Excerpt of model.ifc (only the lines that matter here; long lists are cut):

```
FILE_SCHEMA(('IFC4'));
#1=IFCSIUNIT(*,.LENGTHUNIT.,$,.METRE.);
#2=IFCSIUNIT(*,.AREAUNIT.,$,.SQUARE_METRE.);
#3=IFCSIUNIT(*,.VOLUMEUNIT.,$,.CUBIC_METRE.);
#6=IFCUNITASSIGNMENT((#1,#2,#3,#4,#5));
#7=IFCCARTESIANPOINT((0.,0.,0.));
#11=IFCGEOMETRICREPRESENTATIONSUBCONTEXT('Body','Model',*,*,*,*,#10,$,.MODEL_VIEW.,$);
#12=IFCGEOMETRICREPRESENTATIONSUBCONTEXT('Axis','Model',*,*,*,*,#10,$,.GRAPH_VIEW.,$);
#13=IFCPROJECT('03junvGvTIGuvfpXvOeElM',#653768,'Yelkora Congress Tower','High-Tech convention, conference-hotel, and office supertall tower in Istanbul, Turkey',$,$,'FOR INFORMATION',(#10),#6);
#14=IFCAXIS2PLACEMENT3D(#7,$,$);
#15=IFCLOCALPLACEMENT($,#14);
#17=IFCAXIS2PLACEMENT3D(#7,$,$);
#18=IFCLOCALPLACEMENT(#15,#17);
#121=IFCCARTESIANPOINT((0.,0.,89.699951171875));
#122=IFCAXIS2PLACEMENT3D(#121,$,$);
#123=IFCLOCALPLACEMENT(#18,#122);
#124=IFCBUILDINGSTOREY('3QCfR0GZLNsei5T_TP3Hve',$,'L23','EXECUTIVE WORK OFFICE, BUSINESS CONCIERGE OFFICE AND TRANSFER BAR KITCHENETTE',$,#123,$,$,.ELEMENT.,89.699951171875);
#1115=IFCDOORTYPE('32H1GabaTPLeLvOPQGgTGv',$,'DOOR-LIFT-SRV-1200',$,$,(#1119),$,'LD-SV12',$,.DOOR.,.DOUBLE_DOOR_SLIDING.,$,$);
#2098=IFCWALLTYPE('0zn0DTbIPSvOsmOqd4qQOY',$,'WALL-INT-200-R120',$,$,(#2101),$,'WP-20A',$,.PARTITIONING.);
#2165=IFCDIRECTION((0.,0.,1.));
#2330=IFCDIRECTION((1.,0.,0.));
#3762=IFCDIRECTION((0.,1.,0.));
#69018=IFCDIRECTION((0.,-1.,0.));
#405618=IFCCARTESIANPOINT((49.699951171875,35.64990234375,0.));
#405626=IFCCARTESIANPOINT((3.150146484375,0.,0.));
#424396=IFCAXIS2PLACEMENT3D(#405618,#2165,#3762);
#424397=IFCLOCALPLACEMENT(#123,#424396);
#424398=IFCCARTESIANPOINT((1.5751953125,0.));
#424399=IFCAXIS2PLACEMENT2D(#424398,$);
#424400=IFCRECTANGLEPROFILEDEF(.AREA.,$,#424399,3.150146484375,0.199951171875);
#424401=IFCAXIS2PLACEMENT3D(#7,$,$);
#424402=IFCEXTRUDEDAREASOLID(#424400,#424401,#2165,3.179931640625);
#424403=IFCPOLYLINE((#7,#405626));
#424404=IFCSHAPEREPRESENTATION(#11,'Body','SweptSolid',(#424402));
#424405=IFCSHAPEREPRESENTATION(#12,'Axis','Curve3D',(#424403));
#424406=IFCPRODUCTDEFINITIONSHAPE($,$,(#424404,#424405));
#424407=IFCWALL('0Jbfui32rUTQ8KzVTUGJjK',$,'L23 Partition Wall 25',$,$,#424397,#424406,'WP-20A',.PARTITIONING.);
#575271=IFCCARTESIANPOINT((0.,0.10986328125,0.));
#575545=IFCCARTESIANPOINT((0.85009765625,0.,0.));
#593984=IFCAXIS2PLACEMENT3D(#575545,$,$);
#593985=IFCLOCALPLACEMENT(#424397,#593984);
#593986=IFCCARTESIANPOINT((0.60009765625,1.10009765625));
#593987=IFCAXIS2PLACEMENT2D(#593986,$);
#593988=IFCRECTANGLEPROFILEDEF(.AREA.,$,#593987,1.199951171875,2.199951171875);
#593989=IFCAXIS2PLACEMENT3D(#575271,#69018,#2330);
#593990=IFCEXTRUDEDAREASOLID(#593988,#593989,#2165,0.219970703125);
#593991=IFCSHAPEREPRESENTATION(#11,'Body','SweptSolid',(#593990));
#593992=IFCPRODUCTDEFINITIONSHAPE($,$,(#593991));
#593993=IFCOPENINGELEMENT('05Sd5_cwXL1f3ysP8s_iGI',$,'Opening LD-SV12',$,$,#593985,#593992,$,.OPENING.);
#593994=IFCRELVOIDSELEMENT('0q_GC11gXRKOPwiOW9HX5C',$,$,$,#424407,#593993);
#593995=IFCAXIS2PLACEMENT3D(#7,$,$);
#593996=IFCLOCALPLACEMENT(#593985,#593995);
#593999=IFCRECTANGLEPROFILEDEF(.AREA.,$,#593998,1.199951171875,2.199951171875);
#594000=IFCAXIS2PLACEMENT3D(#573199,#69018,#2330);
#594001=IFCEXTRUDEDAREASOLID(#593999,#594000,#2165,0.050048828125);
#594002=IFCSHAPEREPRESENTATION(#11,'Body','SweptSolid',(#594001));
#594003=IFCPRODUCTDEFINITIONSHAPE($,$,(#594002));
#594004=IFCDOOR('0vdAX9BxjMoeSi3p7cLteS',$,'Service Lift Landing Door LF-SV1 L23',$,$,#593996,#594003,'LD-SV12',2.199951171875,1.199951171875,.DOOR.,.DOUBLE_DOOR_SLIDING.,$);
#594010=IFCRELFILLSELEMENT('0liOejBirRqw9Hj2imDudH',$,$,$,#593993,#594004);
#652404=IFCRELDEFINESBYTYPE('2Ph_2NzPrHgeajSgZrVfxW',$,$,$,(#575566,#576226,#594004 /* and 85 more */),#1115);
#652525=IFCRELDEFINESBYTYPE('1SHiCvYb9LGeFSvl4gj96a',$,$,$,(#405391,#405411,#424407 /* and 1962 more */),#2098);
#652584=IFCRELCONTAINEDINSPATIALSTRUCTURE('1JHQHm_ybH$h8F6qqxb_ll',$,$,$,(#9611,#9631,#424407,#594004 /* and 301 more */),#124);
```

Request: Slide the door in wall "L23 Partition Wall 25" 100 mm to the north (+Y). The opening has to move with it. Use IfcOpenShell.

```python
import ifcopenshell
import ifcopenshell.api.geometry
import ifcopenshell.util.placement

model = ifcopenshell.open("model.ifc")

door = model.by_guid("0vdAX9BxjMoeSi3p7cLteS")
opening = door.FillsVoids[0].RelatingOpeningElement
wall = opening.VoidsElements[0].RelatingBuildingElement

wall_matrix = ifcopenshell.util.placement.get_local_placement(wall.ObjectPlacement)
shift = wall_matrix[:3, 0] * 0.1
before = ifcopenshell.util.placement.get_local_placement(door.ObjectPlacement)[:3, 3].copy()

# The door is placed relative to its opening, so it follows when the opening moves.
matrix = ifcopenshell.util.placement.get_local_placement(opening.ObjectPlacement)
matrix[:3, 3] += shift
ifcopenshell.api.geometry.edit_object_placement(
    model, product=opening, matrix=matrix, is_si=False, should_transform_children=True
)

after = ifcopenshell.util.placement.get_local_placement(door.ObjectPlacement)[:3, 3]
print("door moved by", (after - before).round(3) + 0.0)

model.write("model_updated.ifc")
```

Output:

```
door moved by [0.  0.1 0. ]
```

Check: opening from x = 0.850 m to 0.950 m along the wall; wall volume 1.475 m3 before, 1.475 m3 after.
